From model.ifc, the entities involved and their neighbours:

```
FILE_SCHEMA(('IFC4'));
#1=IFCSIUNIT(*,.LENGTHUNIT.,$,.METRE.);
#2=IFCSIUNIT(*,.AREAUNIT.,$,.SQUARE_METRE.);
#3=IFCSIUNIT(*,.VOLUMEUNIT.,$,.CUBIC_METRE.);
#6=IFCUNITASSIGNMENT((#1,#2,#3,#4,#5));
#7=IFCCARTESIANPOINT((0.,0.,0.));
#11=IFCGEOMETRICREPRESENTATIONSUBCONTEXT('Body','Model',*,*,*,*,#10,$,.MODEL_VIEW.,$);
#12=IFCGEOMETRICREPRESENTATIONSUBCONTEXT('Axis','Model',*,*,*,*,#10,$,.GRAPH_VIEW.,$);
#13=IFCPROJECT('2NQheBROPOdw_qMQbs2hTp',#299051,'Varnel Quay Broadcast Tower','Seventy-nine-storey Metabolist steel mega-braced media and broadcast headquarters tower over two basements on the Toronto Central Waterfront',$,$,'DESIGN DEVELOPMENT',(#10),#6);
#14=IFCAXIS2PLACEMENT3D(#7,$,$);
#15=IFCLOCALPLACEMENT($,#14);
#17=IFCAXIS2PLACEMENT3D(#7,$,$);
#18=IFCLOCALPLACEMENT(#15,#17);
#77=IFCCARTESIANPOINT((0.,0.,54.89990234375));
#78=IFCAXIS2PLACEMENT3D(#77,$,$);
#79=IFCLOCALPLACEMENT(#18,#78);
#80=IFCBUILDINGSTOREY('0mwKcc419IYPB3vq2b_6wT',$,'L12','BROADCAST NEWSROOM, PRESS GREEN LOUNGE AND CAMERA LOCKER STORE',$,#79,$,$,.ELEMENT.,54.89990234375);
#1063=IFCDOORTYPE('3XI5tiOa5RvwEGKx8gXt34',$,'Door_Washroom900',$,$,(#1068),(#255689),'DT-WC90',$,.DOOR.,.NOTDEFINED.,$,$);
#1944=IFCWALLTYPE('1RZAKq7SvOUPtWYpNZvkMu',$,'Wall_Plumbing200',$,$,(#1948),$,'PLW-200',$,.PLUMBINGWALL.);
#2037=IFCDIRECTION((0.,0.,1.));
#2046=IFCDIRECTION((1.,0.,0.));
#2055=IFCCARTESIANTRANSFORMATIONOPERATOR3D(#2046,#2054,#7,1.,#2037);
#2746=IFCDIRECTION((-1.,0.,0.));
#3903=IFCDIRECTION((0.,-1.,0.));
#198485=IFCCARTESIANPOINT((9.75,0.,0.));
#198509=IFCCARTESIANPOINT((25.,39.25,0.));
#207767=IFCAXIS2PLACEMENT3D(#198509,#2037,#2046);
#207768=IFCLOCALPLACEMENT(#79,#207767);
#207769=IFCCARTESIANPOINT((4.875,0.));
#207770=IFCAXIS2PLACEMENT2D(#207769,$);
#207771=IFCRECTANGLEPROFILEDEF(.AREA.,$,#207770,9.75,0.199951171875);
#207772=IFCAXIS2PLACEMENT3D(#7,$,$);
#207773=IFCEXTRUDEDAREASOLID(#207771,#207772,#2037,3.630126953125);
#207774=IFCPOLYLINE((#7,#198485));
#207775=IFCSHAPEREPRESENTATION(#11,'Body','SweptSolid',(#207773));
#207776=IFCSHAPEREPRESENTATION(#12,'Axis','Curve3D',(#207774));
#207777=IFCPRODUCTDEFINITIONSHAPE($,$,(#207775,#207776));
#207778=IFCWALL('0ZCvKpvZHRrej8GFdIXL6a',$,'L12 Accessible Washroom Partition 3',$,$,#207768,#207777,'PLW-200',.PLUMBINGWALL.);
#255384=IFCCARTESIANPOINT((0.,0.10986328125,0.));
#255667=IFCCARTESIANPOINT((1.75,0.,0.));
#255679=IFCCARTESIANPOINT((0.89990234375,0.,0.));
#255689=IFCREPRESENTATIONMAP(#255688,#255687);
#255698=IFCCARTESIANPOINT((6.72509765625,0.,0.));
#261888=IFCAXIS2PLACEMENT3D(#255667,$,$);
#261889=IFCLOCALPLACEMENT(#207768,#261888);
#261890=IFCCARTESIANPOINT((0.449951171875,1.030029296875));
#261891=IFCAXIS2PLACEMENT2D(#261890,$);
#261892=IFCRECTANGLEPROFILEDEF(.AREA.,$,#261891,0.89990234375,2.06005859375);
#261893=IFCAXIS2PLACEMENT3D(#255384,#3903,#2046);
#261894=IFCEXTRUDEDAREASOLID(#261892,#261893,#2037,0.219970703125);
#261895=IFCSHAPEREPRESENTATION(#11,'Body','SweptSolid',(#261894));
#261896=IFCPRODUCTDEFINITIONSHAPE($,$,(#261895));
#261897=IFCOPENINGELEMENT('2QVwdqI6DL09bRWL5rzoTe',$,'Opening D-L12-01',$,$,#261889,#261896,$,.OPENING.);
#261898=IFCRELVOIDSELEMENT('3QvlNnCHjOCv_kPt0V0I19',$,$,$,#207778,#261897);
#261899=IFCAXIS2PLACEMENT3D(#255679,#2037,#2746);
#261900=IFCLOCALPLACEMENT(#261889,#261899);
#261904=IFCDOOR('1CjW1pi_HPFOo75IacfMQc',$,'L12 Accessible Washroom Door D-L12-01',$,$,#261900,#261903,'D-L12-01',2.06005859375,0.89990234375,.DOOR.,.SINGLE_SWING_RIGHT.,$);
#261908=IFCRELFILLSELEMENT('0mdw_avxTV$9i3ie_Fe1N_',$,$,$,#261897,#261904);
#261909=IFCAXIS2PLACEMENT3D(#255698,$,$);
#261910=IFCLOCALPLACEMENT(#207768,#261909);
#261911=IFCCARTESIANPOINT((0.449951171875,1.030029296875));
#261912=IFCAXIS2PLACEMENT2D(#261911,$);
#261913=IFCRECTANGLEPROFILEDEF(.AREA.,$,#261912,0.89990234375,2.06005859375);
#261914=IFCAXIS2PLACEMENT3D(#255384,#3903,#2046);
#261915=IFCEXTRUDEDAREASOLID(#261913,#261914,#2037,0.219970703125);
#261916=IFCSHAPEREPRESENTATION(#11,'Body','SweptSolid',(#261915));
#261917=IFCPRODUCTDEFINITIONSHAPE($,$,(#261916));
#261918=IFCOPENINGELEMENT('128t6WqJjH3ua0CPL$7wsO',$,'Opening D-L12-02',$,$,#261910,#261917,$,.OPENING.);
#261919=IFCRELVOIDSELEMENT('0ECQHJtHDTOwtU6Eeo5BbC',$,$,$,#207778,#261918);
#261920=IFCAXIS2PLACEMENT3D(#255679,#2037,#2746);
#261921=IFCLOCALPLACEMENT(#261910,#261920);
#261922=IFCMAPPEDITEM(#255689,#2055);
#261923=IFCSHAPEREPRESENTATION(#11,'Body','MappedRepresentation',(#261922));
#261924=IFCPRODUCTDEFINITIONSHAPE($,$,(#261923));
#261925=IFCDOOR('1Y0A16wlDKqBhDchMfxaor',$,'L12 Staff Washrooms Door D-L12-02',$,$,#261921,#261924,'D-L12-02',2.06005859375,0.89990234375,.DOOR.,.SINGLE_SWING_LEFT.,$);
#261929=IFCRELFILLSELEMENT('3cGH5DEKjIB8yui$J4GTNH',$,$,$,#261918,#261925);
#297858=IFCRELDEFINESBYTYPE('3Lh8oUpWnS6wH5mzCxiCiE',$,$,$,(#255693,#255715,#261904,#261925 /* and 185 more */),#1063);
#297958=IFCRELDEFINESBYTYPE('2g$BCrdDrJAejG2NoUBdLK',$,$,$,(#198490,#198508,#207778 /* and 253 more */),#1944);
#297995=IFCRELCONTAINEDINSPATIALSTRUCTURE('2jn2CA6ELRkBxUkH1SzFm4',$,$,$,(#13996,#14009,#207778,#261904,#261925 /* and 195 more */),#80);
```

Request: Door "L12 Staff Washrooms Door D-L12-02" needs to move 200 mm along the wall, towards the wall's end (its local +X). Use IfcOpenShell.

```python
import ifcopenshell
import ifcopenshell.api.geometry
import ifcopenshell.util.placement

model = ifcopenshell.open("model.ifc")

door = model.by_guid("1Y0A16wlDKqBhDchMfxaor")
opening = door.FillsVoids[0].RelatingOpeningElement
wall = opening.VoidsElements[0].RelatingBuildingElement

wall_matrix = ifcopenshell.util.placement.get_local_placement(wall.ObjectPlacement)
shift = wall_matrix[:3, 0] * 0.2
before = ifcopenshell.util.placement.get_local_placement(door.ObjectPlacement)[:3, 3].copy()

# The door is placed relative to its opening, so it follows when the opening moves.
matrix = ifcopenshell.util.placement.get_local_placement(opening.ObjectPlacement)
matrix[:3, 3] += shift
ifcopenshell.api.geometry.edit_object_placement(
    model, product=opening, matrix=matrix, is_si=False, should_transform_children=True
)

after = ifcopenshell.util.placement.get_local_placement(door.ObjectPlacement)[:3, 3]
print("door moved by", (after - before).round(3) + 0.0)

model.write("model_updated.ifc")
```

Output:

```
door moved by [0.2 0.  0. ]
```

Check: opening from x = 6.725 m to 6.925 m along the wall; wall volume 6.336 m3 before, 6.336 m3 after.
